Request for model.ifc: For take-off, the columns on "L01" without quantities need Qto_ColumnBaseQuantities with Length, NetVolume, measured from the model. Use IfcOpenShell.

First a look at what the model holds.

```python
import ifcopenshell
import ifcopenshell.util.element
import ifcopenshell.util.unit

model = ifcopenshell.open("model.ifc")
print(model.schema)
for unit_type in ("LENGTHUNIT", "AREAUNIT", "VOLUMEUNIT"):
    print(unit_type, ifcopenshell.util.unit.calculate_unit_scale(model, unit_type))
storey = next(s for s in model.by_type("IfcBuildingStorey") if s.Name == "L01")
columns = [e for e in ifcopenshell.util.element.get_decomposition(storey) if e.is_a("IfcColumn")]
for e in sorted(columns, key=lambda e: e.id()):
    print(e.id(), e.is_a(), e.Name, list(ifcopenshell.util.element.get_psets(e, qtos_only=True)), sep=" | ")
```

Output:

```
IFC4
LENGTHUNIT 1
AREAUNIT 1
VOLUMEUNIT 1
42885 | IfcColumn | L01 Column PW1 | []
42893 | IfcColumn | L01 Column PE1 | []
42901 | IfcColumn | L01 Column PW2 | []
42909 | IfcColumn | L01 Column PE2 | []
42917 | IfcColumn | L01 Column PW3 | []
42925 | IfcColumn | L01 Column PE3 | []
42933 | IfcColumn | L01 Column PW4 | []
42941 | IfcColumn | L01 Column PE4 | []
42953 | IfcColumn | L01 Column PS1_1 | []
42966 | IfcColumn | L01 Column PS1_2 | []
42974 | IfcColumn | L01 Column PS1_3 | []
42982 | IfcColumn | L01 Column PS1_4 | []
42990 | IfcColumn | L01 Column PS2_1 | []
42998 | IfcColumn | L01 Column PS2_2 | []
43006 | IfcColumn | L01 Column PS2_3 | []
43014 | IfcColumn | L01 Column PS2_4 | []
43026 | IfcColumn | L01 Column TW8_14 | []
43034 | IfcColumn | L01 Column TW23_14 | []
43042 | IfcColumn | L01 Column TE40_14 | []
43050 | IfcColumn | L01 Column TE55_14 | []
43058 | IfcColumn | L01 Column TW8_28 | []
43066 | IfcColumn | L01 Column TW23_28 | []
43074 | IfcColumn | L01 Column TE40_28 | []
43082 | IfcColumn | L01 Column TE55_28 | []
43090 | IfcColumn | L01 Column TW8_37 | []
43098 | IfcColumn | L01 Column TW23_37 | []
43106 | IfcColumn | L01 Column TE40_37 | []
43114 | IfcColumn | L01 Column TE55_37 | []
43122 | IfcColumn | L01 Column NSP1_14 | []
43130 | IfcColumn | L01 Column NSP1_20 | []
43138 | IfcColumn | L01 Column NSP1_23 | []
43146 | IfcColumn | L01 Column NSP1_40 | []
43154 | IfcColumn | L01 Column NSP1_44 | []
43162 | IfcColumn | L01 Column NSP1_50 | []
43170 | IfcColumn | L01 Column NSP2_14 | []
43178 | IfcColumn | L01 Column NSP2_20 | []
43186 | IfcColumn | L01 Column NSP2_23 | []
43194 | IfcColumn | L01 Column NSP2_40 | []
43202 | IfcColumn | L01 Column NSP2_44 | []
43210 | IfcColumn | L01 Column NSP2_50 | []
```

```python
import ifcopenshell
import ifcopenshell.api.pset
import ifcopenshell.geom
import ifcopenshell.util.element
import ifcopenshell.util.shape
import ifcopenshell.util.unit

model = ifcopenshell.open("model.ifc")
unit_scale = ifcopenshell.util.unit.calculate_unit_scale(model)
volume_scale = ifcopenshell.util.unit.calculate_unit_scale(model, "VOLUMEUNIT")
settings = ifcopenshell.geom.settings()

storey = next(s for s in model.by_type("IfcBuildingStorey") if s.Name == "L01")
columns = [e for e in ifcopenshell.util.element.get_decomposition(storey) if e.is_a("IfcColumn")]

for e in sorted(columns, key=lambda e: e.id()):
    if ifcopenshell.util.element.get_psets(e, qtos_only=True, should_inherit=False):
        continue
    # Geometry comes back in metres, in the element's own axes.
    shape = ifcopenshell.geom.create_shape(settings, e)
    values = {
        "Length": ifcopenshell.util.shape.get_z(shape.geometry) / unit_scale,
        "NetVolume": ifcopenshell.util.shape.get_volume(shape.geometry) / volume_scale,
    }
    qto = ifcopenshell.api.pset.add_qto(model, product=e, name="Qto_ColumnBaseQuantities")
    ifcopenshell.api.pset.edit_qto(model, qto=qto, properties=values)
    print(e.id(), {k: round(v, 3) for k, v in values.items()})

model.write("model_v2.ifc")
```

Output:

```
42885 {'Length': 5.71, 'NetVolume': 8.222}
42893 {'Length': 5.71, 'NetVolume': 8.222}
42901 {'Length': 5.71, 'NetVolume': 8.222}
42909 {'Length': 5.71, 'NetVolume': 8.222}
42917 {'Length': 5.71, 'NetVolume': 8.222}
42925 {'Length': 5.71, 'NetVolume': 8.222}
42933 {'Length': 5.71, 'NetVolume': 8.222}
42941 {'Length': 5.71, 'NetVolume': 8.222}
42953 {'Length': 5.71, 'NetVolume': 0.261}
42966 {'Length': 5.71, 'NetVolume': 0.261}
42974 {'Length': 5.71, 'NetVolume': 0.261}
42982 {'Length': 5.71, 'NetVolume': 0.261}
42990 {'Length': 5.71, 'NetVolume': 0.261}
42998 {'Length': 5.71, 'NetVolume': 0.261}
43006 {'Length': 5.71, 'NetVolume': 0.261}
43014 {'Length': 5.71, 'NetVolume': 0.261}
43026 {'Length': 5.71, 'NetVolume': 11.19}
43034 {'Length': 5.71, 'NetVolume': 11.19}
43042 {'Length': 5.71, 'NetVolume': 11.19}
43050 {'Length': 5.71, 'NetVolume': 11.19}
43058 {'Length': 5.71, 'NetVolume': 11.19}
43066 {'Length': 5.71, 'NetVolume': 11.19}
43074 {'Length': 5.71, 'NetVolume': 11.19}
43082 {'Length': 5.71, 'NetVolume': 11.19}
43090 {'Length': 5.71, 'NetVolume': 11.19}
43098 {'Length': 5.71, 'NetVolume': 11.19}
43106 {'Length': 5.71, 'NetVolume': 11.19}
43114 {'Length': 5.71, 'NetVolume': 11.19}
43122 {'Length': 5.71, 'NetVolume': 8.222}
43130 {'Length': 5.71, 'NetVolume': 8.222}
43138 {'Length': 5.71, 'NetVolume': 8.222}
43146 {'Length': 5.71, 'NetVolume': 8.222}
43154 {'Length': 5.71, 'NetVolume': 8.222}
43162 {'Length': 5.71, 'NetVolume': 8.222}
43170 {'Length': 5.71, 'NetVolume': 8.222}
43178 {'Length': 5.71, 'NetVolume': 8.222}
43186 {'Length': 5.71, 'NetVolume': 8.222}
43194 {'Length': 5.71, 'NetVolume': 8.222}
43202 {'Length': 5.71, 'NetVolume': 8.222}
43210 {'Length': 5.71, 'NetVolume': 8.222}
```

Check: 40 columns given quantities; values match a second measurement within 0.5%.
